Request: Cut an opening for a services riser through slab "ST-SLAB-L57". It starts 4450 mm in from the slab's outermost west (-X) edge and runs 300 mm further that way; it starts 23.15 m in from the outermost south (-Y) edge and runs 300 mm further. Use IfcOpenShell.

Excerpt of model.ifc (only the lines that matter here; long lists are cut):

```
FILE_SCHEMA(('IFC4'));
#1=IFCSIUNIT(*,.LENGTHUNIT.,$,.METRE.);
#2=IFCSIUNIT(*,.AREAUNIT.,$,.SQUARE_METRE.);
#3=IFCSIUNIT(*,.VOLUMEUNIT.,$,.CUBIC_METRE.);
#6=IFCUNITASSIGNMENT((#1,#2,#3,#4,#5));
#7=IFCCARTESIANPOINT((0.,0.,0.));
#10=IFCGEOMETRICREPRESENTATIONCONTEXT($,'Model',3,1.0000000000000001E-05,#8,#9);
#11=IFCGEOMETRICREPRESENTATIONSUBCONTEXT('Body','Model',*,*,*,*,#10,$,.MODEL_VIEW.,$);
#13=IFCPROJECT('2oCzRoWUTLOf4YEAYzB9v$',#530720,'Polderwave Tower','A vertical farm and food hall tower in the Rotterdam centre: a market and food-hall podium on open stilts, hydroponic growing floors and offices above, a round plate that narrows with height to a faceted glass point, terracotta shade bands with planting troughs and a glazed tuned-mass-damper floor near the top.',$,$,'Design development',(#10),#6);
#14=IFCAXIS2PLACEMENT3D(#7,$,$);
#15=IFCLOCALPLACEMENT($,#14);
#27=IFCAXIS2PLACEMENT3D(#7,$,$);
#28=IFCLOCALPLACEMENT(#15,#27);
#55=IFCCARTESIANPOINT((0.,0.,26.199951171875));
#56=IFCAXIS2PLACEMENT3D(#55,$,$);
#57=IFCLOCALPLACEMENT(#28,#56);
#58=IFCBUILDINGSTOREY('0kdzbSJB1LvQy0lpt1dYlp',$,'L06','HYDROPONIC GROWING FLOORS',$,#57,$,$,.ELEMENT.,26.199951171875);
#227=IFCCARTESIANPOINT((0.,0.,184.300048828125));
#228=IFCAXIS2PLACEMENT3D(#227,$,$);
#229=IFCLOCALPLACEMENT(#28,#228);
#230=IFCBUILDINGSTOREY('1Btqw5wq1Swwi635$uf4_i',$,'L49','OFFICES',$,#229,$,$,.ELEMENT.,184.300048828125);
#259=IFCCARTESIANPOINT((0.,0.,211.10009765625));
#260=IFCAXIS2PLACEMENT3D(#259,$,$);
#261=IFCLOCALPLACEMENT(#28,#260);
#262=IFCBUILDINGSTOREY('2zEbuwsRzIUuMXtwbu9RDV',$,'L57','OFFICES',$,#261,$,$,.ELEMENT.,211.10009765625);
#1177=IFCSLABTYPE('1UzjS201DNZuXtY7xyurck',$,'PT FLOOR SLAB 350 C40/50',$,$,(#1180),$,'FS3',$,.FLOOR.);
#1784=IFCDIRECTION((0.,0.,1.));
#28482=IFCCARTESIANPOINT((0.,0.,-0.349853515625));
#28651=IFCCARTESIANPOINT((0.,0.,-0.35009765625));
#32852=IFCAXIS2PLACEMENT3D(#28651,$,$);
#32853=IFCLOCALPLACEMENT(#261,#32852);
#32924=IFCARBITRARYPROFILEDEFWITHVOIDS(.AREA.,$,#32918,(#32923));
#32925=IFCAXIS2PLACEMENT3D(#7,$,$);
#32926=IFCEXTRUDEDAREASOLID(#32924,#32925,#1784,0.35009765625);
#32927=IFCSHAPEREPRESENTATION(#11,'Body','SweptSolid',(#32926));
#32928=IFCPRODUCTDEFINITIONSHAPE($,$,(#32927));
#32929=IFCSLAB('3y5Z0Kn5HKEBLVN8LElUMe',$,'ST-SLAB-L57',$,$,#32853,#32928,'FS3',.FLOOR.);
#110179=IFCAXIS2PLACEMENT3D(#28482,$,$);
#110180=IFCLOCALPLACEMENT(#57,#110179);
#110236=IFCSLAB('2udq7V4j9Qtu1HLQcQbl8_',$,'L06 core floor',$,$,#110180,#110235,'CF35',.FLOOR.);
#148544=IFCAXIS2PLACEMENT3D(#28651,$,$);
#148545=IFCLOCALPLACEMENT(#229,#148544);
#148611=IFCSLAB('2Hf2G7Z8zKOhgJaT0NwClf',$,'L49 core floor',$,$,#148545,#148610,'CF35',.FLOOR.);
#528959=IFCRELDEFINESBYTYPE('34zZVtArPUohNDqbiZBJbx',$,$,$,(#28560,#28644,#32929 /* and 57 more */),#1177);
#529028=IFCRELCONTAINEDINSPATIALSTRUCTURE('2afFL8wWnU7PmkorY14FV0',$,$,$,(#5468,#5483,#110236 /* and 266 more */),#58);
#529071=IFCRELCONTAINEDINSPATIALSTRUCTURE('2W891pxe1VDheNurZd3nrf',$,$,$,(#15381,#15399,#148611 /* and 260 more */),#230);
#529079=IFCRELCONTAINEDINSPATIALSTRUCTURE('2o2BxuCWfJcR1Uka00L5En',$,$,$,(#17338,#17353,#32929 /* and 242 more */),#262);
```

```python
import numpy as np
import ifcopenshell
import ifcopenshell.api.feature
import ifcopenshell.api.geometry
import ifcopenshell.api.root
import ifcopenshell.geom
import ifcopenshell.util.placement
import ifcopenshell.util.representation
import ifcopenshell.util.shape
import ifcopenshell.util.unit

model = ifcopenshell.open("model.ifc")
unit_scale = ifcopenshell.util.unit.calculate_unit_scale(model)
settings = ifcopenshell.geom.settings()


def volume(element):
    """Net volume in cubic metres, openings subtracted."""
    shape = ifcopenshell.geom.create_shape(settings, element)
    return ifcopenshell.util.shape.get_volume(shape.geometry)


slab = model.by_guid("3y5Z0Kn5HKEBLVN8LElUMe")
before = volume(slab)

# Extent in the slab's own axes, in metres. The edges named are its -X and -Y sides.
slab_shape = ifcopenshell.geom.create_shape(settings, slab)
vertices = ifcopenshell.util.shape.get_vertices(slab_shape.geometry)
x_min, y_min, bottom = vertices.min(axis=0)
top = vertices[:, 2].max()

opening = ifcopenshell.api.root.create_entity(model, ifc_class="IfcOpeningElement", name="Services riser opening", predefined_type="OPENING")
context = ifcopenshell.util.representation.get_context(model, "Model", "Body", "MODEL_VIEW")
width, depth = 0.3, 0.3
outline = [(0.0, 0.0), (width, 0.0), (width, depth), (0.0, depth), (0.0, 0.0)]
# Overshoot both faces by 50 mm so the cut is clean.
shape = ifcopenshell.api.geometry.add_slab_representation(
    model, context=context, depth=top - bottom + 0.1, polyline=outline
)
ifcopenshell.api.geometry.assign_representation(model, product=opening, representation=shape)

matrix = ifcopenshell.util.placement.get_local_placement(slab.ObjectPlacement)
matrix[:, 3] = matrix @ np.append(np.array([x_min + 4.45, y_min + 23.15, bottom - 0.05]) / unit_scale, 1.0)
ifcopenshell.api.geometry.edit_object_placement(model, product=opening, matrix=matrix, is_si=False)
ifcopenshell.api.feature.add_feature(model, feature=opening, element=slab)

after = volume(slab)

print(f"slab volume {before:.3f} -> {after:.3f} m3")

model.write("model_v2.ifc")
```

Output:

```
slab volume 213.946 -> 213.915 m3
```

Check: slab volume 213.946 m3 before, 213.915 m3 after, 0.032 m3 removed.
